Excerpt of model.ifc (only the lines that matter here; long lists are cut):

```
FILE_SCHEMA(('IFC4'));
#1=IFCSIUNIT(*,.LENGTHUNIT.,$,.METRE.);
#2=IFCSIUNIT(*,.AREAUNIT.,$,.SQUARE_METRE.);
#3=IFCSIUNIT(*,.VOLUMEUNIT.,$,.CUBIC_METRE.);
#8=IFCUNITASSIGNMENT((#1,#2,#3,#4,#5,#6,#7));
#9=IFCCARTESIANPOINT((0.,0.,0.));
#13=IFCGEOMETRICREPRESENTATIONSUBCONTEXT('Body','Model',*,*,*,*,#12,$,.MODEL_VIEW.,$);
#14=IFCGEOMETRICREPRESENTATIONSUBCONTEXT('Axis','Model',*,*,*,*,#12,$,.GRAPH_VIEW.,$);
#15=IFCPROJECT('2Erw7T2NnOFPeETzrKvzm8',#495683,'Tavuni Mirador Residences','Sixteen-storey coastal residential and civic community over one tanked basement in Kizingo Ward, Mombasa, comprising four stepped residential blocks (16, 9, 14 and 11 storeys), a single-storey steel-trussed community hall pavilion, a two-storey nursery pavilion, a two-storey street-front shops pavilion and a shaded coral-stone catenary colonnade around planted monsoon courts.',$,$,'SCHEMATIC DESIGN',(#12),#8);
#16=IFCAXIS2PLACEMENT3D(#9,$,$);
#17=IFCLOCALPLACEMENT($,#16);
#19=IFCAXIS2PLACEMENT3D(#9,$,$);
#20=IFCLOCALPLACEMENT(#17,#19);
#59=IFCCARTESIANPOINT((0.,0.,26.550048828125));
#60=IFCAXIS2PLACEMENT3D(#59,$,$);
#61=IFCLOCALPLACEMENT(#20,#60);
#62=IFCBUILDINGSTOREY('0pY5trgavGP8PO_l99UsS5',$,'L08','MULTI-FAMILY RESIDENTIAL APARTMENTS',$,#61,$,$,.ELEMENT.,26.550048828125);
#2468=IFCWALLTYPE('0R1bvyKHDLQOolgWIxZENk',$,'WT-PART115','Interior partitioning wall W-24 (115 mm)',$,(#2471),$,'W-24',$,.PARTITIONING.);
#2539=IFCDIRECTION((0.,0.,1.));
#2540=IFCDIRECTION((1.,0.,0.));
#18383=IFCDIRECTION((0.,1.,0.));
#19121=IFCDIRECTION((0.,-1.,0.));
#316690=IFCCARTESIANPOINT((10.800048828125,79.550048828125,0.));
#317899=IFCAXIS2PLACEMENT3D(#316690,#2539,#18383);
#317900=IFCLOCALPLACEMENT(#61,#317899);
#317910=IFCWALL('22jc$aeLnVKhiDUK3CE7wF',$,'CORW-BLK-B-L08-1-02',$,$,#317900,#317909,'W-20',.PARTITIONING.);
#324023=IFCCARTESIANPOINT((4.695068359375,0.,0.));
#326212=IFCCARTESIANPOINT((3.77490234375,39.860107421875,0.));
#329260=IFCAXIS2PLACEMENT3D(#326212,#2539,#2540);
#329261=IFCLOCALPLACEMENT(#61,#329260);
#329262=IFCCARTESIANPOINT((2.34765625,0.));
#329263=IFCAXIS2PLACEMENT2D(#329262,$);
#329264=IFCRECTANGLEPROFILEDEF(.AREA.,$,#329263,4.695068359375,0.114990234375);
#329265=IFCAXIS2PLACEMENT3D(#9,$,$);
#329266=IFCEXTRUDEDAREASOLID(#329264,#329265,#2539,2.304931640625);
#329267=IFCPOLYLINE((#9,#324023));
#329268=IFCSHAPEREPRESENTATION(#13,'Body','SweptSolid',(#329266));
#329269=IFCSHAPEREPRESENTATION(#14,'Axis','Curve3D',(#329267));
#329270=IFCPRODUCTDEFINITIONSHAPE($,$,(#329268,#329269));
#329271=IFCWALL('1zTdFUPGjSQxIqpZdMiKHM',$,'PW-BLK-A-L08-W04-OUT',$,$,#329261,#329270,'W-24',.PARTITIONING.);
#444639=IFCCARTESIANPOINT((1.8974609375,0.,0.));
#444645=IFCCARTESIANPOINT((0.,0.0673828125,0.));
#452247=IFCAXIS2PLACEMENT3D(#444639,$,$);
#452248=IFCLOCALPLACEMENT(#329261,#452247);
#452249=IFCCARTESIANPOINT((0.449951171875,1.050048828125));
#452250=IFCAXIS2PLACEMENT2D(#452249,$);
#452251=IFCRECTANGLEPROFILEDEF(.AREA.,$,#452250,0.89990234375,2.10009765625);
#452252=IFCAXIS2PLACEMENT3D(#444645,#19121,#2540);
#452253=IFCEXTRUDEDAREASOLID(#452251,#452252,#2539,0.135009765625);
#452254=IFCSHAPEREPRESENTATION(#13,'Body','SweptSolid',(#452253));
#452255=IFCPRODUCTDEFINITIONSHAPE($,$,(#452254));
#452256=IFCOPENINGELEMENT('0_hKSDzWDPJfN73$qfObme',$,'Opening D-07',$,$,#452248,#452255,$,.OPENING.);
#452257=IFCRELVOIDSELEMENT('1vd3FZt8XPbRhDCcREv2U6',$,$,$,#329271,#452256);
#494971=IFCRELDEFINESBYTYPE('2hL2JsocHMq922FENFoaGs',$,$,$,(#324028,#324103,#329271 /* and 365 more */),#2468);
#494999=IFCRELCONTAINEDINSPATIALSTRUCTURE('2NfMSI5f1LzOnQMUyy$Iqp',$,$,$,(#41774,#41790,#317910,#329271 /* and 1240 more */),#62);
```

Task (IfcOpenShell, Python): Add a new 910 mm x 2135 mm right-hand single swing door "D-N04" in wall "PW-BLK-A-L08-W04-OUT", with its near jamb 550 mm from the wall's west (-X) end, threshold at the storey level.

```python
import numpy as np
import ifcopenshell
import ifcopenshell.api.feature
import ifcopenshell.api.geometry
import ifcopenshell.api.root
import ifcopenshell.api.spatial
import ifcopenshell.geom
import ifcopenshell.util.element
import ifcopenshell.util.placement
import ifcopenshell.util.representation
import ifcopenshell.util.shape
import ifcopenshell.util.unit

model = ifcopenshell.open("model.ifc")
unit_scale = ifcopenshell.util.unit.calculate_unit_scale(model)
settings = ifcopenshell.geom.settings()


def volume(element):
    """Net volume in cubic metres, openings subtracted."""
    shape = ifcopenshell.geom.create_shape(settings, element)
    return ifcopenshell.util.shape.get_volume(shape.geometry)


wall = model.by_guid("1zTdFUPGjSQxIqpZdMiKHM")
storey = ifcopenshell.util.element.get_container(wall, ifc_class="IfcBuildingStorey")
context = ifcopenshell.util.representation.get_context(model, "Model", "Body", "MODEL_VIEW")
before = volume(wall)

width, height, from_end, sill = 0.91, 2.135, 0.55, 0.0  # metres

# The wall runs along its own X axis, and the end named is its -X end.
wall_shape = ifcopenshell.geom.create_shape(settings, wall)
x, y, z = ifcopenshell.util.shape.get_vertices(wall_shape.geometry).T
start = x.min() + from_end
face, thickness = float(y.min()), float(y.max() - y.min())
wall_matrix = ifcopenshell.util.placement.get_local_placement(wall.ObjectPlacement)
level = ifcopenshell.util.placement.get_local_placement(storey.ObjectPlacement)[2, 3]


def in_wall(x, y):
    """Placement at x, y metres in the wall's axes, at sill height."""
    matrix = wall_matrix.copy()
    matrix[:, 3] = wall_matrix @ np.array([x / unit_scale, y / unit_scale, 0.0, 1.0])
    matrix[2, 3] = level + sill / unit_scale
    return matrix


# Opening: a box that overshoots both wall faces by 50 mm.
opening = ifcopenshell.api.root.create_entity(model, ifc_class="IfcOpeningElement", predefined_type="OPENING")
box = ifcopenshell.api.geometry.add_wall_representation(
    model, context=context, length=width, height=height, thickness=thickness + 0.1
)
ifcopenshell.api.geometry.assign_representation(model, product=opening, representation=box)
ifcopenshell.api.geometry.edit_object_placement(model, product=opening, matrix=in_wall(start, face - 0.05), is_si=False)
ifcopenshell.api.feature.add_feature(model, feature=opening, element=wall)

door = ifcopenshell.api.root.create_entity(model, ifc_class="IfcDoor", name="D-N04", predefined_type="DOOR")
door.OverallWidth, door.OverallHeight = width / unit_scale, height / unit_scale
door.OperationType = "SINGLE_SWING_RIGHT"
body = ifcopenshell.api.geometry.add_door_representation(
    model,
    context=context,
    overall_width=door.OverallWidth,
    overall_height=door.OverallHeight,
    operation_type="SINGLE_SWING_RIGHT",
    lining_properties={"LiningDepth": thickness / unit_scale, "ThresholdDepth": thickness / unit_scale},
)
ifcopenshell.api.geometry.assign_representation(model, product=door, representation=body)
ifcopenshell.api.spatial.assign_container(model, products=[door], relating_structure=storey)
ifcopenshell.api.feature.add_filling(model, opening=opening, element=door)

# The lining spans the wall, so the door starts at the wall face.
ifcopenshell.api.geometry.edit_object_placement(model, product=door, matrix=in_wall(start, face), is_si=False)

after = volume(wall)

print(f"wall volume {before:.3f} -> {after:.3f} m3")

model.write("model_updated.ifc")
```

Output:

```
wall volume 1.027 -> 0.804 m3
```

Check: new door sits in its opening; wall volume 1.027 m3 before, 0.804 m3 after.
